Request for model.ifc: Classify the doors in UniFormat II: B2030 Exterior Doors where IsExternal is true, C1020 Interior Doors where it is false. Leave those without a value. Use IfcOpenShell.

First a look at what the model holds.

```python
import ifcopenshell
import ifcopenshell.util.element

model = ifcopenshell.open("model.ifc")
print(model.schema)
print("classifications:", [c.Name for c in model.by_type("IfcClassification")])
values = [ifcopenshell.util.element.get_pset(e, "Pset_DoorCommon", "IsExternal") for e in model.by_type("IfcDoor")]
for value in (True, False, None):
    print("IsExternal", value, values.count(value))
```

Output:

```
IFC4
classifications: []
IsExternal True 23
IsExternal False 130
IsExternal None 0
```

```python
import ifcopenshell
import ifcopenshell.api.classification
import ifcopenshell.util.element

model = ifcopenshell.open("model.ifc")

system = ifcopenshell.api.classification.add_classification(model, classification="UniFormat II")

doors = model.by_type("IfcDoor")
external = {e: ifcopenshell.util.element.get_pset(e, "Pset_DoorCommon", "IsExternal") for e in doors}
for flag, code, name in ((True, "B2030", "Exterior Doors"), (False, "C1020", "Interior Doors")):
    products = [e for e in doors if external[e] is flag]
    ifcopenshell.api.classification.add_reference(
        model, products=products, classification=system, identification=code, name=name
    )
    print(code, len(products))

model.write("model_rev.ifc")
```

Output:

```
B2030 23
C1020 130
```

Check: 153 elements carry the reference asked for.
